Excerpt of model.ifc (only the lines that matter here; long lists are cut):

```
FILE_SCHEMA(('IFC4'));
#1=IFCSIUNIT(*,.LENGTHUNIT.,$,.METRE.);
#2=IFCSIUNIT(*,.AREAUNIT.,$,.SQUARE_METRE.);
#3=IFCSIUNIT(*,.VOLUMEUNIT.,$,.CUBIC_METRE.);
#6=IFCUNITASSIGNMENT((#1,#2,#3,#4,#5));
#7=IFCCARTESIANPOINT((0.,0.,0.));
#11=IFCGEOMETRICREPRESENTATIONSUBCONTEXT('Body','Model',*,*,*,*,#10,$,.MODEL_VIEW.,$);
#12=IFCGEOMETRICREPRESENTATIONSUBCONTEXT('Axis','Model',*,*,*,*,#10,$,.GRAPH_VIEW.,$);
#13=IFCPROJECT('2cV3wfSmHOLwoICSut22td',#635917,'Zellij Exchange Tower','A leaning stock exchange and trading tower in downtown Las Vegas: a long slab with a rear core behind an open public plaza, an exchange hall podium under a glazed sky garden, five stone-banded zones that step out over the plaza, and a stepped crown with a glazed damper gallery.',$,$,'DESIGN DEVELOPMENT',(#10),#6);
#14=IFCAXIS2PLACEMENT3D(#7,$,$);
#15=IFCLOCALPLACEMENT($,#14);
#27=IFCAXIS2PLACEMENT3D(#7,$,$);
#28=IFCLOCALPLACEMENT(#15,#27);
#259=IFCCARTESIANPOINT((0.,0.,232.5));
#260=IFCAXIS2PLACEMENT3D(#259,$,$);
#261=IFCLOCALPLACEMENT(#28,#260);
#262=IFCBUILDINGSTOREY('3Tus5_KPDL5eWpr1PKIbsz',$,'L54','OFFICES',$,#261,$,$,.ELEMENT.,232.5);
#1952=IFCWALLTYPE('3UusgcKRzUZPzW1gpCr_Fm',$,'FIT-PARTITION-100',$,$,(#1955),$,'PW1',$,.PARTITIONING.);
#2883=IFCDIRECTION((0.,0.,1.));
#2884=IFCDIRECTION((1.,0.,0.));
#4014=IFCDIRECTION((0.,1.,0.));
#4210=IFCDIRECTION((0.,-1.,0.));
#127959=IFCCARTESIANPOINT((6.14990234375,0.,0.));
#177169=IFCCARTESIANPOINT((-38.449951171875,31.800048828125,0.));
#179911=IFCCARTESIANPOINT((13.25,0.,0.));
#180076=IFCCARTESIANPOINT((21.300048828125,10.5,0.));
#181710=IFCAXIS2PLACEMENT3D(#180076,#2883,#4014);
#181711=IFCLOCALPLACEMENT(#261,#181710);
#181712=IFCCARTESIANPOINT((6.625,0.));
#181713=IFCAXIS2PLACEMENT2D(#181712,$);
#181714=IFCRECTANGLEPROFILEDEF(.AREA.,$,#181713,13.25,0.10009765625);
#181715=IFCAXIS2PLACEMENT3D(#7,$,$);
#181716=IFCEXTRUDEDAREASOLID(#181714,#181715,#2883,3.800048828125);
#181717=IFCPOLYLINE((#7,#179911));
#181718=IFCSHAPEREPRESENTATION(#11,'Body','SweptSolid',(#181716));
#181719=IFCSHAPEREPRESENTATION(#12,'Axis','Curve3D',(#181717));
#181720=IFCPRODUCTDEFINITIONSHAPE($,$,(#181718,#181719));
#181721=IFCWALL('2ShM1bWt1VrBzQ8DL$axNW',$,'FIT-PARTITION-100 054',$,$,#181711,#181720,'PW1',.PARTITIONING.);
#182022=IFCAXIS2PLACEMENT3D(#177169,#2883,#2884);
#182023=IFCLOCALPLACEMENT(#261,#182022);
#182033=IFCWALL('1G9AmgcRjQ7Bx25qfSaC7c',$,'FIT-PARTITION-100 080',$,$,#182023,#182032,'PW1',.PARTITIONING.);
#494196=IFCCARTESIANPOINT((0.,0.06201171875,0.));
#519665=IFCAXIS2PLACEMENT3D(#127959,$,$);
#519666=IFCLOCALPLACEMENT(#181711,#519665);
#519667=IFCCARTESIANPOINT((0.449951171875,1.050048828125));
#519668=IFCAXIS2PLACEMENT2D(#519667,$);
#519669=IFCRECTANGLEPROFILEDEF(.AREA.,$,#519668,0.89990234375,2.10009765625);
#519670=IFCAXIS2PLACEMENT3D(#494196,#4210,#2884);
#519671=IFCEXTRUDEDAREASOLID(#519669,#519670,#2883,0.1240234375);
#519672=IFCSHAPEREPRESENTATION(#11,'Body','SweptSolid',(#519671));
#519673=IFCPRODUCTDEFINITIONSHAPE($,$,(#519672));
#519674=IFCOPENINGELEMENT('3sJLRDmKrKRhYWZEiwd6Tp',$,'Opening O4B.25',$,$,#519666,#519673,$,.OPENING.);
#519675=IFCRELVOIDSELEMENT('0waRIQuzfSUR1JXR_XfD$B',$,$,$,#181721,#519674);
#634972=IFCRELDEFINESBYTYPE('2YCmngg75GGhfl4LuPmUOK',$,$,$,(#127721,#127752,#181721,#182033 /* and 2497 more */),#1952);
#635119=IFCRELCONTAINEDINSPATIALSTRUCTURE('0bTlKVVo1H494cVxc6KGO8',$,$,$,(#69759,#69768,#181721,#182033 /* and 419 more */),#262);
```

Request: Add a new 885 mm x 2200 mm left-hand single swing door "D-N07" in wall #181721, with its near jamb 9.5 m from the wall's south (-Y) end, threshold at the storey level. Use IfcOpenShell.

```python
import numpy as np
import ifcopenshell
import ifcopenshell.api.feature
import ifcopenshell.api.geometry
import ifcopenshell.api.root
import ifcopenshell.api.spatial
import ifcopenshell.geom
import ifcopenshell.util.element
import ifcopenshell.util.placement
import ifcopenshell.util.representation
import ifcopenshell.util.shape
import ifcopenshell.util.unit

model = ifcopenshell.open("model.ifc")
unit_scale = ifcopenshell.util.unit.calculate_unit_scale(model)
settings = ifcopenshell.geom.settings()


def volume(element):
    """Net volume in cubic metres, openings subtracted."""
    shape = ifcopenshell.geom.create_shape(settings, element)
    return ifcopenshell.util.shape.get_volume(shape.geometry)


wall = model.by_id(181721)
storey = ifcopenshell.util.element.get_container(wall, ifc_class="IfcBuildingStorey")
context = ifcopenshell.util.representation.get_context(model, "Model", "Body", "MODEL_VIEW")
before = volume(wall)

width, height, from_end, sill = 0.885, 2.2, 9.5, 0.0  # metres

# The wall runs along its own X axis, and the end named is its -X end.
wall_shape = ifcopenshell.geom.create_shape(settings, wall)
x, y, z = ifcopenshell.util.shape.get_vertices(wall_shape.geometry).T
start = x.min() + from_end
face, thickness = float(y.min()), float(y.max() - y.min())
wall_matrix = ifcopenshell.util.placement.get_local_placement(wall.ObjectPlacement)
level = ifcopenshell.util.placement.get_local_placement(storey.ObjectPlacement)[2, 3]


def in_wall(x, y):
    """Placement at x, y metres in the wall's axes, at sill height."""
    matrix = wall_matrix.copy()
    matrix[:, 3] = wall_matrix @ np.array([x / unit_scale, y / unit_scale, 0.0, 1.0])
    matrix[2, 3] = level + sill / unit_scale
    return matrix


# Opening: a box that overshoots both wall faces by 50 mm.
opening = ifcopenshell.api.root.create_entity(model, ifc_class="IfcOpeningElement", predefined_type="OPENING")
box = ifcopenshell.api.geometry.add_wall_representation(
    model, context=context, length=width, height=height, thickness=thickness + 0.1
)
ifcopenshell.api.geometry.assign_representation(model, product=opening, representation=box)
ifcopenshell.api.geometry.edit_object_placement(model, product=opening, matrix=in_wall(start, face - 0.05), is_si=False)
ifcopenshell.api.feature.add_feature(model, feature=opening, element=wall)

door = ifcopenshell.api.root.create_entity(model, ifc_class="IfcDoor", name="D-N07", predefined_type="DOOR")
door.OverallWidth, door.OverallHeight = width / unit_scale, height / unit_scale
door.OperationType = "SINGLE_SWING_LEFT"
body = ifcopenshell.api.geometry.add_door_representation(
    model,
    context=context,
    overall_width=door.OverallWidth,
    overall_height=door.OverallHeight,
    operation_type="SINGLE_SWING_LEFT",
    lining_properties={"LiningDepth": thickness / unit_scale, "ThresholdDepth": thickness / unit_scale},
)
ifcopenshell.api.geometry.assign_representation(model, product=door, representation=body)
ifcopenshell.api.spatial.assign_container(model, products=[door], relating_structure=storey)
ifcopenshell.api.feature.add_filling(model, opening=opening, element=door)

# The lining spans the wall, so the door starts at the wall face.
ifcopenshell.api.geometry.edit_object_placement(model, product=door, matrix=in_wall(start, face), is_si=False)

after = volume(wall)

print(f"wall volume {before:.3f} -> {after:.3f} m3")

model.write("model_updated.ifc")
```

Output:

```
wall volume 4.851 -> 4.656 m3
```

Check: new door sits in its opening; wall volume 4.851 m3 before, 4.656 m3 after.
